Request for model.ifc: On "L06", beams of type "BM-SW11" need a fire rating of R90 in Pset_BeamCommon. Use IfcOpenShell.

First a look at what the model holds.

```python
import ifcopenshell
import ifcopenshell.util.element

model = ifcopenshell.open("model.ifc")
print(model.schema)
storey = next(s for s in model.by_type("IfcBuildingStorey") if s.Name == "L06")
beams = [e for e in ifcopenshell.util.element.get_decomposition(storey) if e.is_a("IfcBeam")]
seen = {}
for e in beams:
    element_type = ifcopenshell.util.element.get_type(e)
    key = (element_type.Name if element_type != e and element_type else None, ifcopenshell.util.element.get_pset(e, "Pset_BeamCommon", "FireRating"))
    seen[key] = seen.get(key, 0) + 1
for (name, value), count in sorted(seen.items(), key=str):
    print(count, "x", name, "|", value)
```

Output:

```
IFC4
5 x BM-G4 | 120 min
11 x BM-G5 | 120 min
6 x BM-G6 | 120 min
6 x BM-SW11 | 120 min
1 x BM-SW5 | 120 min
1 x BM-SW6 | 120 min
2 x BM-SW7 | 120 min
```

```python
import ifcopenshell
import ifcopenshell.api.pset
import ifcopenshell.util.element

model = ifcopenshell.open("model.ifc")

storey = next(s for s in model.by_type("IfcBuildingStorey") if s.Name == "L06")
beams = [e for e in ifcopenshell.util.element.get_decomposition(storey) if e.is_a("IfcBeam")]

count = 0
for e in beams:
    element_type = ifcopenshell.util.element.get_type(e)
    if element_type in (None, e) or element_type.Name != "BM-SW11":
        continue
    # add_pset returns the element's existing set when there is one.
    pset = ifcopenshell.api.pset.add_pset(model, product=e, name="Pset_BeamCommon")
    ifcopenshell.api.pset.edit_pset(model, pset=pset, properties={"FireRating": "R90"})
    count += 1

print(count, "beams updated")

model.write("model-out.ifc")
```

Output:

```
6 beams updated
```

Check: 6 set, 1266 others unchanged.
